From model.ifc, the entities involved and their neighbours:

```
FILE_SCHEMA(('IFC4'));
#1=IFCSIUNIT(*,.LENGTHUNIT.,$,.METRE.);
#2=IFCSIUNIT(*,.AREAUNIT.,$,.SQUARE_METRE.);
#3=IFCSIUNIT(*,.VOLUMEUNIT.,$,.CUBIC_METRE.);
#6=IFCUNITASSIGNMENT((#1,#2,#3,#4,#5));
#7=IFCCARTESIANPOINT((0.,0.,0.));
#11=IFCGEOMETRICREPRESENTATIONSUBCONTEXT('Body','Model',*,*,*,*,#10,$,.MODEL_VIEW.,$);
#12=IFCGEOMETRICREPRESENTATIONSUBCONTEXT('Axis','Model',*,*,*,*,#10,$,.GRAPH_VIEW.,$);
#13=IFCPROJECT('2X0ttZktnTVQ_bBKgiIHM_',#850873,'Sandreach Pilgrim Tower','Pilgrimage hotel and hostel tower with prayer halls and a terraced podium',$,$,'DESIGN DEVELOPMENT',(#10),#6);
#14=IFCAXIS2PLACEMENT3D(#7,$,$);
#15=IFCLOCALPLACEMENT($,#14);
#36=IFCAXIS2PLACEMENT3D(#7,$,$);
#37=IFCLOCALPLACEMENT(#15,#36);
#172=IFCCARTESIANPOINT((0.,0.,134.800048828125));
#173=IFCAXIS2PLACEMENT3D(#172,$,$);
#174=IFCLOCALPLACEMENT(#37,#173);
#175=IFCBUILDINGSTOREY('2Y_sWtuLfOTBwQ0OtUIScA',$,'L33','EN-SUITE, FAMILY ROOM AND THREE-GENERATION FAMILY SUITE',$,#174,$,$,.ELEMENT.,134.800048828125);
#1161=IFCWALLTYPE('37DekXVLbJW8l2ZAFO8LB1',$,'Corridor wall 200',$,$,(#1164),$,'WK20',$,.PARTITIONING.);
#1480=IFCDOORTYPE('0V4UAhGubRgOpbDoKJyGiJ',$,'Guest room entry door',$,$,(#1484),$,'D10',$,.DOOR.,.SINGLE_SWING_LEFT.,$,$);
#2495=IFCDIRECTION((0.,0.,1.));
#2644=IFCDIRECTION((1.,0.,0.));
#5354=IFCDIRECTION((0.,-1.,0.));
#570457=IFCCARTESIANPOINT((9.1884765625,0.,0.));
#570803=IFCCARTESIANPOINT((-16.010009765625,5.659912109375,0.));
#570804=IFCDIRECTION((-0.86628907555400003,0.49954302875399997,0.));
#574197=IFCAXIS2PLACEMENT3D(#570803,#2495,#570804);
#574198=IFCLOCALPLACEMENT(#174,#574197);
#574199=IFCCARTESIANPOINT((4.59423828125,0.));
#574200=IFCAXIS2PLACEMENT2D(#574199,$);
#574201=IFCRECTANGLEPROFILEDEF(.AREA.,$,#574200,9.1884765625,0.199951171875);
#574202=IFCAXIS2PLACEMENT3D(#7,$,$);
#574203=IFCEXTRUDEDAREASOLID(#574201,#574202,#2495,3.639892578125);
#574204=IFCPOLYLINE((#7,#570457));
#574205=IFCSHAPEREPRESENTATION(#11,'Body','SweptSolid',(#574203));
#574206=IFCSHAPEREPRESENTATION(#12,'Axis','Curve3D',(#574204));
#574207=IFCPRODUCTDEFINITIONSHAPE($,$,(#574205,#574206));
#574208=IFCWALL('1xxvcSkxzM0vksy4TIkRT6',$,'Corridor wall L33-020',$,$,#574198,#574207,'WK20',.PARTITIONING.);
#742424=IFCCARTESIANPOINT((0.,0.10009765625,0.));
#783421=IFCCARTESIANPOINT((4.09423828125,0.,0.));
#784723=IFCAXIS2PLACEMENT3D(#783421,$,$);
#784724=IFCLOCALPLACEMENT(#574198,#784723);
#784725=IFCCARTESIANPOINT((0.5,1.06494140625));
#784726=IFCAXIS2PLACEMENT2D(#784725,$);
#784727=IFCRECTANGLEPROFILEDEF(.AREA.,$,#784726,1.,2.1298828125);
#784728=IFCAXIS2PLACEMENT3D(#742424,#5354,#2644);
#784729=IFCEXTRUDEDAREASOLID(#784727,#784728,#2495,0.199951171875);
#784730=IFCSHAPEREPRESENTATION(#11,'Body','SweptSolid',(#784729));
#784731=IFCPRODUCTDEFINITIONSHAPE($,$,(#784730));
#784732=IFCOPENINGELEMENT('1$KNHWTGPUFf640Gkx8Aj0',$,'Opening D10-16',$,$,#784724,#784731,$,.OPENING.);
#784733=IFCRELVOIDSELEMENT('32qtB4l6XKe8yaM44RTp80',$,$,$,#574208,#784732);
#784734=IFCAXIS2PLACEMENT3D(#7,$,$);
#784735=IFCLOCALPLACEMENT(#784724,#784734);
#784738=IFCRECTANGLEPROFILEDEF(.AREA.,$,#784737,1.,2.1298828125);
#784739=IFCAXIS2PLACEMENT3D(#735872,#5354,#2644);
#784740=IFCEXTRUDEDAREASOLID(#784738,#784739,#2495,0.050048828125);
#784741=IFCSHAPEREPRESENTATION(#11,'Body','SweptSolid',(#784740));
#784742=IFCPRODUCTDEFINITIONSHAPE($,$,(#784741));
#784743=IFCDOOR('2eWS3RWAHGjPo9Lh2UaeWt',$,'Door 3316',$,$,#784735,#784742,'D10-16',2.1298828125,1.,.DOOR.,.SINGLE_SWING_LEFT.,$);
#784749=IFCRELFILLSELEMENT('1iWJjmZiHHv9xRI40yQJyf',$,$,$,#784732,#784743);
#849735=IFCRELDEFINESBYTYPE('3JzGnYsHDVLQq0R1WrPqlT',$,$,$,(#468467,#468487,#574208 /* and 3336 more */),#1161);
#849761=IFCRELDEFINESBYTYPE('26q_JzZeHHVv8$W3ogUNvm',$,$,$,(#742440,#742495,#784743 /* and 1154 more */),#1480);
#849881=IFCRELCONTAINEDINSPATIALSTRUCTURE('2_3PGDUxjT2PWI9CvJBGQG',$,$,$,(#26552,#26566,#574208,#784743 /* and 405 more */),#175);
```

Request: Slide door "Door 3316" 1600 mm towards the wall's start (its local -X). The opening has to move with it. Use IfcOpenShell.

```python
import ifcopenshell
import ifcopenshell.api.geometry
import ifcopenshell.util.placement
import ifcopenshell.util.unit

model = ifcopenshell.open("model.ifc")
unit_scale = ifcopenshell.util.unit.calculate_unit_scale(model)

door = model.by_guid("2eWS3RWAHGjPo9Lh2UaeWt")
opening = door.FillsVoids[0].RelatingOpeningElement
wall = opening.VoidsElements[0].RelatingBuildingElement

wall_matrix = ifcopenshell.util.placement.get_local_placement(wall.ObjectPlacement)
shift = wall_matrix[:3, 0] * -1.6 / unit_scale
before = ifcopenshell.util.placement.get_local_placement(door.ObjectPlacement)[:3, 3].copy()

# The door is placed relative to its opening, so it follows when the opening moves.
matrix = ifcopenshell.util.placement.get_local_placement(opening.ObjectPlacement)
matrix[:3, 3] += shift
ifcopenshell.api.geometry.edit_object_placement(
    model, product=opening, matrix=matrix, is_si=False, should_transform_children=True
)

after = ifcopenshell.util.placement.get_local_placement(door.ObjectPlacement)[:3, 3]
print("door moved by", (after - before).round(3) + 0.0)

model.write("model-out.ifc")
```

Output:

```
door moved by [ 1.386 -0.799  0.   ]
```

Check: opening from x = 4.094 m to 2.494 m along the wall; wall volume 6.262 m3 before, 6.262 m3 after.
